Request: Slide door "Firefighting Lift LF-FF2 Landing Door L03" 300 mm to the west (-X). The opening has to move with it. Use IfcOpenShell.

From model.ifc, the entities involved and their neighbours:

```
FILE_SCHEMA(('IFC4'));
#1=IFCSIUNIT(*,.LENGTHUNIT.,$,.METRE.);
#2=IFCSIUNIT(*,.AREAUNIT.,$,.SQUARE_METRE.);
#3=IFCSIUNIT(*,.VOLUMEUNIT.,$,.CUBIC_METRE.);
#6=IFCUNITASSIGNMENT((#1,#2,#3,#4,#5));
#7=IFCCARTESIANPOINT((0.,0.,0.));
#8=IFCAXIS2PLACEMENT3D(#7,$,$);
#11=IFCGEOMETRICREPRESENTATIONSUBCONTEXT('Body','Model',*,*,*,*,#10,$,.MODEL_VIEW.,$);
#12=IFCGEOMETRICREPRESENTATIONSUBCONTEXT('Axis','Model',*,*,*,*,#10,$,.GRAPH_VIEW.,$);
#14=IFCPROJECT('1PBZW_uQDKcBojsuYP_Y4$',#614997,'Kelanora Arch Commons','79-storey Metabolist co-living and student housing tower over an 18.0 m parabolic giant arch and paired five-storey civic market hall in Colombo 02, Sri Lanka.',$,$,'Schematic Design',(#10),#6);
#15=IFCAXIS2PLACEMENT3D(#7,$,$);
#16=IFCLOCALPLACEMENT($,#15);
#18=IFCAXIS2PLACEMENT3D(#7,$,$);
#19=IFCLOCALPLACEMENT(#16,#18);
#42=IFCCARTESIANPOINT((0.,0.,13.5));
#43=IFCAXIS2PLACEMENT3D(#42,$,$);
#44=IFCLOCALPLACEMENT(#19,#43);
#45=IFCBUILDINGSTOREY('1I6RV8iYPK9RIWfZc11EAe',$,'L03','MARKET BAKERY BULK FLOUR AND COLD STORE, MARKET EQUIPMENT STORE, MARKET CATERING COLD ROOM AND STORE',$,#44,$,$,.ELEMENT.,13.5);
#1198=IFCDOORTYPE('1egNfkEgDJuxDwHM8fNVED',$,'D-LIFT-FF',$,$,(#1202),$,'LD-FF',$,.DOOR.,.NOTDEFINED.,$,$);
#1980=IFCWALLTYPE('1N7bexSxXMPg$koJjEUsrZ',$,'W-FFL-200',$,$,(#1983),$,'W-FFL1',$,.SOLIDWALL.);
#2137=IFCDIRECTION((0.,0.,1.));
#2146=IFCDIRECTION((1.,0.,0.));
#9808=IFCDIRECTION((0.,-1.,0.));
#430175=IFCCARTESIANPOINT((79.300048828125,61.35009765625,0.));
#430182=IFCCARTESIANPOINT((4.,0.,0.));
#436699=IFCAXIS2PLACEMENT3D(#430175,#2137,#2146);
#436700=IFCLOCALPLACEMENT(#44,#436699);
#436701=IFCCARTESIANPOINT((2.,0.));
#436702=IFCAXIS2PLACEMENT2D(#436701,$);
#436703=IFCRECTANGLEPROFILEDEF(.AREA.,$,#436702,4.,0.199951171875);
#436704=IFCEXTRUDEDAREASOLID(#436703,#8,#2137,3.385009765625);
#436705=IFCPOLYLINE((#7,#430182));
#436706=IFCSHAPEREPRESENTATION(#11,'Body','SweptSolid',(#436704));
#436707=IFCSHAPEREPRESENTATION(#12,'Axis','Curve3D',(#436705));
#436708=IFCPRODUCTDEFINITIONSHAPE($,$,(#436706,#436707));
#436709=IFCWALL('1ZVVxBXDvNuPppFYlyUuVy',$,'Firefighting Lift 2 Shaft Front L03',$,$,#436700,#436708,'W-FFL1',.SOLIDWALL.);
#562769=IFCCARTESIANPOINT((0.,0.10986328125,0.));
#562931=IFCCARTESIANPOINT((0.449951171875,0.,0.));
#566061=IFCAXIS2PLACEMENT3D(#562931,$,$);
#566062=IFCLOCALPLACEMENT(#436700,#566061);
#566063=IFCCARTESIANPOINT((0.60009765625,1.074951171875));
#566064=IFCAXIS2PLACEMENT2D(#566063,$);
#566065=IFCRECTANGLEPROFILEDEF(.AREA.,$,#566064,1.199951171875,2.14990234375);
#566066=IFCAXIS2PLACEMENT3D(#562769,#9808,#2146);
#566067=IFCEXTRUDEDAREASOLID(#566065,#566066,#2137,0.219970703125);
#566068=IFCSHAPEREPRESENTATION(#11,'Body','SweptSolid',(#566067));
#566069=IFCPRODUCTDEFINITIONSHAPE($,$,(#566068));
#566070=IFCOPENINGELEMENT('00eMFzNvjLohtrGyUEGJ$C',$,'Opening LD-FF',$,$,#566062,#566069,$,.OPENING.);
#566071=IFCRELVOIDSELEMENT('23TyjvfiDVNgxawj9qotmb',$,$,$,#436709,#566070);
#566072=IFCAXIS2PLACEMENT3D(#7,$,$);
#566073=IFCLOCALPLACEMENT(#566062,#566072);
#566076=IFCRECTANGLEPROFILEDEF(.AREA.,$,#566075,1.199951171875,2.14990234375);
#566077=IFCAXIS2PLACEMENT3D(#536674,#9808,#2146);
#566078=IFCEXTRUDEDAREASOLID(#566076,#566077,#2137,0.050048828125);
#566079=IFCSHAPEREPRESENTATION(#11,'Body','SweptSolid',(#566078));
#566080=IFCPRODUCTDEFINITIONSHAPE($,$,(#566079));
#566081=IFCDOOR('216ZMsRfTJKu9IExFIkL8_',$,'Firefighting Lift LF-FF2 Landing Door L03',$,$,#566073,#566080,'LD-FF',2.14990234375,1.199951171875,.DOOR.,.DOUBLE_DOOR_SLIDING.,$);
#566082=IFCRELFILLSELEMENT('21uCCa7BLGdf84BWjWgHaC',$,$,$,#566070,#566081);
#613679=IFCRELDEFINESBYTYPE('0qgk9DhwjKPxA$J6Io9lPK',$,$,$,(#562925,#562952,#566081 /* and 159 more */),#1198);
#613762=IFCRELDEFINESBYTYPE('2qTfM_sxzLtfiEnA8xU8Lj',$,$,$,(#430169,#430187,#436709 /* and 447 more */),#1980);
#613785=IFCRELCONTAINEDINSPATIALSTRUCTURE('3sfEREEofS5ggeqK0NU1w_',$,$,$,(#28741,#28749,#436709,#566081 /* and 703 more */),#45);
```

```python
import ifcopenshell
import ifcopenshell.api.geometry
import ifcopenshell.util.placement

model = ifcopenshell.open("model.ifc")

door = model.by_guid("216ZMsRfTJKu9IExFIkL8_")
opening = door.FillsVoids[0].RelatingOpeningElement
wall = opening.VoidsElements[0].RelatingBuildingElement

wall_matrix = ifcopenshell.util.placement.get_local_placement(wall.ObjectPlacement)
shift = wall_matrix[:3, 0] * -0.3
before = ifcopenshell.util.placement.get_local_placement(door.ObjectPlacement)[:3, 3].copy()

# The door is placed relative to its opening, so it follows when the opening moves.
matrix = ifcopenshell.util.placement.get_local_placement(opening.ObjectPlacement)
matrix[:3, 3] += shift
ifcopenshell.api.geometry.edit_object_placement(
    model, product=opening, matrix=matrix, is_si=False, should_transform_children=True
)

after = ifcopenshell.util.placement.get_local_placement(door.ObjectPlacement)[:3, 3]
print("door moved by", (after - before).round(3) + 0.0)

model.write("model_edited.ifc")
```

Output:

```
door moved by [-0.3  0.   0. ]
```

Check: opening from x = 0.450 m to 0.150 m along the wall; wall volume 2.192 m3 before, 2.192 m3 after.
